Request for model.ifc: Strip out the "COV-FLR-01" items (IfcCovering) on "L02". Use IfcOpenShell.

First a look at what the model holds.

```python
import ifcopenshell
import ifcopenshell.util.element

model = ifcopenshell.open("model.ifc")
print(model.schema)
storey = next(s for s in model.by_type("IfcBuildingStorey") if s.Name == "L02")
coverings = [e for e in ifcopenshell.util.element.get_decomposition(storey) if e.is_a("IfcCovering")]
seen = {}
for e in coverings:
    element_type = ifcopenshell.util.element.get_type(e)
    name = element_type.Name if element_type not in (None, e) else None
    seen[name] = seen.get(name, 0) + 1
for name, count in sorted(seen.items(), key=str):
    print(count, "x", name)
```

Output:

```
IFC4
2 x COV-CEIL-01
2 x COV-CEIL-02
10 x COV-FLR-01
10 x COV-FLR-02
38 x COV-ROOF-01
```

```python
import ifcopenshell
import ifcopenshell.api.root
import ifcopenshell.util.element

model = ifcopenshell.open("model.ifc")

storey = next(s for s in model.by_type("IfcBuildingStorey") if s.Name == "L02")
coverings = [e for e in ifcopenshell.util.element.get_decomposition(storey) if e.is_a("IfcCovering")]
targets = [e for e in coverings if (t := ifcopenshell.util.element.get_type(e)) not in (None, e) and t.Name == "COV-FLR-01"]

for e in targets:
    ifcopenshell.api.root.remove_product(model, product=e)
print(len(targets), "removed")

model.write("model_rev.ifc")
```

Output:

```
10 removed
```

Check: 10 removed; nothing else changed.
